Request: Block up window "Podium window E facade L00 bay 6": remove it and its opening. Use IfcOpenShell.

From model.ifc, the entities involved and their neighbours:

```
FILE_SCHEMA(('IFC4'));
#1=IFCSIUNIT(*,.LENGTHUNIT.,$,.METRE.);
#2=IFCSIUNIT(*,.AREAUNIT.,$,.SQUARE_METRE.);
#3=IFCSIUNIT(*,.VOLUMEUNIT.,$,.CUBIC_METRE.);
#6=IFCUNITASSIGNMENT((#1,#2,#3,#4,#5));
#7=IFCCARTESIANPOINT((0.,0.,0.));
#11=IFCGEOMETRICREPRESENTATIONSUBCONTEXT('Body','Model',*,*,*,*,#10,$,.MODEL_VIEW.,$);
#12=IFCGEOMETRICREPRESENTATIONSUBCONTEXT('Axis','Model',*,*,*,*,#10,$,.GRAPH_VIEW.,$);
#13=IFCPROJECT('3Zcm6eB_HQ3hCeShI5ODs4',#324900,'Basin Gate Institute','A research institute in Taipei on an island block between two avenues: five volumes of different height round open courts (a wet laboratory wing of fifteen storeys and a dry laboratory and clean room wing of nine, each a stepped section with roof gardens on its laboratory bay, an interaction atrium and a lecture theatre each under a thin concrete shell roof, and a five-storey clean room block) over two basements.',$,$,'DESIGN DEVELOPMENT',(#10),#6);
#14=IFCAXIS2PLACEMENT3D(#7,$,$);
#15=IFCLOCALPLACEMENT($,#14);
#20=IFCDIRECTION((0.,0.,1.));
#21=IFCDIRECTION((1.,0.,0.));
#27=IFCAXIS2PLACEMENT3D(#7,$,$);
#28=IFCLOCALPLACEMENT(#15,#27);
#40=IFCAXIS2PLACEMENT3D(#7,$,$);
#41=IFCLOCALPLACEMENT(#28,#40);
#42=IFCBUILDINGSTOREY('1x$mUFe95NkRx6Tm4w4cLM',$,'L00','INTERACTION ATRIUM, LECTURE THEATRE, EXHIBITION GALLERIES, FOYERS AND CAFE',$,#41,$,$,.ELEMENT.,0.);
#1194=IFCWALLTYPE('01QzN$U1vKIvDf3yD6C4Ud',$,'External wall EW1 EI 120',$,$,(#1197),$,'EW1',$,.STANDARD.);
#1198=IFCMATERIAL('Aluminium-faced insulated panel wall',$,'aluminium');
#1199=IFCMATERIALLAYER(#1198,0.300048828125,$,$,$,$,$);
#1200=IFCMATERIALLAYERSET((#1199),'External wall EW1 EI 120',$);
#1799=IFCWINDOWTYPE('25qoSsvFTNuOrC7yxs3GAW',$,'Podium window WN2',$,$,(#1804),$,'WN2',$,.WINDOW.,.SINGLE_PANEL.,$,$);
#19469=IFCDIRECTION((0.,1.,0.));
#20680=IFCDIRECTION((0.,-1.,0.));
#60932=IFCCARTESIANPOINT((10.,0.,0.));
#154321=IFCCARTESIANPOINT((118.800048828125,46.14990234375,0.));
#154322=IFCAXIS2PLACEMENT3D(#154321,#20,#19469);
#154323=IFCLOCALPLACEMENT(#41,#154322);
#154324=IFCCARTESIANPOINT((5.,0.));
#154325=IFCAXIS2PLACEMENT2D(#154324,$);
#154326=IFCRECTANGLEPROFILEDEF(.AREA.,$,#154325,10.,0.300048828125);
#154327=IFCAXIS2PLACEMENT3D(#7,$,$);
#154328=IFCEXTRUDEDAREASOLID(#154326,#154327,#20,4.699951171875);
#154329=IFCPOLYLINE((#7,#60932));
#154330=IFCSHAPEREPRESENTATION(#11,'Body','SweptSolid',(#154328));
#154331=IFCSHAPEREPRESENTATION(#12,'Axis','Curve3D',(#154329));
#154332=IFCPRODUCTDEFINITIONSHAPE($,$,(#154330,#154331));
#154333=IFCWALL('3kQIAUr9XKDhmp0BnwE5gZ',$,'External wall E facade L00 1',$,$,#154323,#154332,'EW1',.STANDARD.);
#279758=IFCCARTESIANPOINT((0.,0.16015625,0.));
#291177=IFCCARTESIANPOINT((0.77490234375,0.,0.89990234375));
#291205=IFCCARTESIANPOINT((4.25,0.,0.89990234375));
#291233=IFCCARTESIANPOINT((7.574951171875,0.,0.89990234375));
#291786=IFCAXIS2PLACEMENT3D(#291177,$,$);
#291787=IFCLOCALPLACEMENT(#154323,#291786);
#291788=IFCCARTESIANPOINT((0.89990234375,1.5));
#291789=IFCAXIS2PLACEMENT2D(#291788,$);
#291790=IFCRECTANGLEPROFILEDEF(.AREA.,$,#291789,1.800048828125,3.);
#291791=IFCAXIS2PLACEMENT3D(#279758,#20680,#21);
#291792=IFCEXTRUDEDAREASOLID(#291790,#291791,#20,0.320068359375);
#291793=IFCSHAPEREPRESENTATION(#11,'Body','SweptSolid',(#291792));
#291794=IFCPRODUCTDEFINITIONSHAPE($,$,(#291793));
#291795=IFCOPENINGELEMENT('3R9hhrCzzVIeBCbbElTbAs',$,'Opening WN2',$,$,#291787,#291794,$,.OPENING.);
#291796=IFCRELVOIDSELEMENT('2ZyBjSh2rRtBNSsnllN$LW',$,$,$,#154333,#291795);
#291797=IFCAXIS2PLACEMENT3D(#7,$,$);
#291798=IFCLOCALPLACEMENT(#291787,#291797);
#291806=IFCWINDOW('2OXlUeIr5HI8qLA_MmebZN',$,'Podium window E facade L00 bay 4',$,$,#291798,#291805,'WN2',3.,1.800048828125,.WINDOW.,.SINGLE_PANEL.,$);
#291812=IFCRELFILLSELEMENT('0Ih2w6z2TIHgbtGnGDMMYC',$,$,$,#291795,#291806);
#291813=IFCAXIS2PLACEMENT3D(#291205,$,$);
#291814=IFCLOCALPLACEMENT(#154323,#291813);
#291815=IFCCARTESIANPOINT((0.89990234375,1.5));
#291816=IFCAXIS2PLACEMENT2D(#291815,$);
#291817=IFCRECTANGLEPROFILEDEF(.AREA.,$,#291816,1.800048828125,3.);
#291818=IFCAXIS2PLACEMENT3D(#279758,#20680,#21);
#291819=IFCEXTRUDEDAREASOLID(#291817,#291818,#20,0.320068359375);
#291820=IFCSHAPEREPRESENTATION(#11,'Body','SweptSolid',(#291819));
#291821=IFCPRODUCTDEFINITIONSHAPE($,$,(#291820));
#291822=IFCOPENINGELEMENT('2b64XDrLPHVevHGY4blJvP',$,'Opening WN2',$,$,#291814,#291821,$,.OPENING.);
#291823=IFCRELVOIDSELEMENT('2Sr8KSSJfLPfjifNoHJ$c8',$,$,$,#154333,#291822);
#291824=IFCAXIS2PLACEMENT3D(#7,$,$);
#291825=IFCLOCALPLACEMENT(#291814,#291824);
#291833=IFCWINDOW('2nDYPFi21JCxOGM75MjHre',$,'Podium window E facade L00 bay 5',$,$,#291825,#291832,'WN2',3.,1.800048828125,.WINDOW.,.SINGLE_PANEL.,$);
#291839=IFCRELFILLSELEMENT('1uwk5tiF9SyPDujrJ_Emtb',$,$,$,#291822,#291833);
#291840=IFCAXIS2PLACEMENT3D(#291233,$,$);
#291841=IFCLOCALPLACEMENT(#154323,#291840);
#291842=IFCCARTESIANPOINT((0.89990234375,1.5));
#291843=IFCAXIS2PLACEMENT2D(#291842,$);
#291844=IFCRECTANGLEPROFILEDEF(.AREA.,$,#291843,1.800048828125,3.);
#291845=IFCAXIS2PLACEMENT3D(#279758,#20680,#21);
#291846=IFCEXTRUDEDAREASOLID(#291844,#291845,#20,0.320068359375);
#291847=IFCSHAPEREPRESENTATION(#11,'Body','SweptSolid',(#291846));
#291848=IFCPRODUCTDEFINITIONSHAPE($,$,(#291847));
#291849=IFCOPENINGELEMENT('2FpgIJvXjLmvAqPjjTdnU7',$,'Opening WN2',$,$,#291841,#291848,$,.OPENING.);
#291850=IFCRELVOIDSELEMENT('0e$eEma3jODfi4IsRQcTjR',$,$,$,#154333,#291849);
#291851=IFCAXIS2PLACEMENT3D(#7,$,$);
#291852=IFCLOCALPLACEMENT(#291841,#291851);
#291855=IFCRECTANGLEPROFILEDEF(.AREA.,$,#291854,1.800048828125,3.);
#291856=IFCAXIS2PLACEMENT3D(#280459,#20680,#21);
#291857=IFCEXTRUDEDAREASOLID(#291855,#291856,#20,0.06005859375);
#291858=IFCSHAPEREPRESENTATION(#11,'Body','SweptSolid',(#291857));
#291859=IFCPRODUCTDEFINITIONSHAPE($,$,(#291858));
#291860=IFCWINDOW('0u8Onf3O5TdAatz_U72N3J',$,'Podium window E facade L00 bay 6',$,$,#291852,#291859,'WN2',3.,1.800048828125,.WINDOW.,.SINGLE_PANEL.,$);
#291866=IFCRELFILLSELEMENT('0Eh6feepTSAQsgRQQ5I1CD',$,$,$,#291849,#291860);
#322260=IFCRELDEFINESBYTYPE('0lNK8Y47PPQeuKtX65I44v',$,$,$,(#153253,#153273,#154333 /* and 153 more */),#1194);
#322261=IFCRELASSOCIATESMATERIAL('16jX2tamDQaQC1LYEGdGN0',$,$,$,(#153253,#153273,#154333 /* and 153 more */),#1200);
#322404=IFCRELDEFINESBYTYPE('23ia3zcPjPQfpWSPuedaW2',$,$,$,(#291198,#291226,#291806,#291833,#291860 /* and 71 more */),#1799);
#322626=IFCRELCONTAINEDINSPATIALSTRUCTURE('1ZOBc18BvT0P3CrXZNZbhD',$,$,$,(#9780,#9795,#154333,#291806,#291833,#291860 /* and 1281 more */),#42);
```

```python
import ifcopenshell
import ifcopenshell.api.feature
import ifcopenshell.api.root
import ifcopenshell.geom
import ifcopenshell.util.shape

model = ifcopenshell.open("model.ifc")
settings = ifcopenshell.geom.settings()


def volume(element):
    """Net volume in cubic metres, openings subtracted."""
    shape = ifcopenshell.geom.create_shape(settings, element)
    return ifcopenshell.util.shape.get_volume(shape.geometry)


window = model.by_id(291860)
opening = window.FillsVoids[0].RelatingOpeningElement
wall = opening.VoidsElements[0].RelatingBuildingElement
before = volume(wall)

ifcopenshell.api.root.remove_product(model, product=window)
ifcopenshell.api.feature.remove_feature(model, feature=opening)

after = volume(wall)

print(f"wall volume {before:.3f} -> {after:.3f} m3")

model.write("model_v2.ifc")
```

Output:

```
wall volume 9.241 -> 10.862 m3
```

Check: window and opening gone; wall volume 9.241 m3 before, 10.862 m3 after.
